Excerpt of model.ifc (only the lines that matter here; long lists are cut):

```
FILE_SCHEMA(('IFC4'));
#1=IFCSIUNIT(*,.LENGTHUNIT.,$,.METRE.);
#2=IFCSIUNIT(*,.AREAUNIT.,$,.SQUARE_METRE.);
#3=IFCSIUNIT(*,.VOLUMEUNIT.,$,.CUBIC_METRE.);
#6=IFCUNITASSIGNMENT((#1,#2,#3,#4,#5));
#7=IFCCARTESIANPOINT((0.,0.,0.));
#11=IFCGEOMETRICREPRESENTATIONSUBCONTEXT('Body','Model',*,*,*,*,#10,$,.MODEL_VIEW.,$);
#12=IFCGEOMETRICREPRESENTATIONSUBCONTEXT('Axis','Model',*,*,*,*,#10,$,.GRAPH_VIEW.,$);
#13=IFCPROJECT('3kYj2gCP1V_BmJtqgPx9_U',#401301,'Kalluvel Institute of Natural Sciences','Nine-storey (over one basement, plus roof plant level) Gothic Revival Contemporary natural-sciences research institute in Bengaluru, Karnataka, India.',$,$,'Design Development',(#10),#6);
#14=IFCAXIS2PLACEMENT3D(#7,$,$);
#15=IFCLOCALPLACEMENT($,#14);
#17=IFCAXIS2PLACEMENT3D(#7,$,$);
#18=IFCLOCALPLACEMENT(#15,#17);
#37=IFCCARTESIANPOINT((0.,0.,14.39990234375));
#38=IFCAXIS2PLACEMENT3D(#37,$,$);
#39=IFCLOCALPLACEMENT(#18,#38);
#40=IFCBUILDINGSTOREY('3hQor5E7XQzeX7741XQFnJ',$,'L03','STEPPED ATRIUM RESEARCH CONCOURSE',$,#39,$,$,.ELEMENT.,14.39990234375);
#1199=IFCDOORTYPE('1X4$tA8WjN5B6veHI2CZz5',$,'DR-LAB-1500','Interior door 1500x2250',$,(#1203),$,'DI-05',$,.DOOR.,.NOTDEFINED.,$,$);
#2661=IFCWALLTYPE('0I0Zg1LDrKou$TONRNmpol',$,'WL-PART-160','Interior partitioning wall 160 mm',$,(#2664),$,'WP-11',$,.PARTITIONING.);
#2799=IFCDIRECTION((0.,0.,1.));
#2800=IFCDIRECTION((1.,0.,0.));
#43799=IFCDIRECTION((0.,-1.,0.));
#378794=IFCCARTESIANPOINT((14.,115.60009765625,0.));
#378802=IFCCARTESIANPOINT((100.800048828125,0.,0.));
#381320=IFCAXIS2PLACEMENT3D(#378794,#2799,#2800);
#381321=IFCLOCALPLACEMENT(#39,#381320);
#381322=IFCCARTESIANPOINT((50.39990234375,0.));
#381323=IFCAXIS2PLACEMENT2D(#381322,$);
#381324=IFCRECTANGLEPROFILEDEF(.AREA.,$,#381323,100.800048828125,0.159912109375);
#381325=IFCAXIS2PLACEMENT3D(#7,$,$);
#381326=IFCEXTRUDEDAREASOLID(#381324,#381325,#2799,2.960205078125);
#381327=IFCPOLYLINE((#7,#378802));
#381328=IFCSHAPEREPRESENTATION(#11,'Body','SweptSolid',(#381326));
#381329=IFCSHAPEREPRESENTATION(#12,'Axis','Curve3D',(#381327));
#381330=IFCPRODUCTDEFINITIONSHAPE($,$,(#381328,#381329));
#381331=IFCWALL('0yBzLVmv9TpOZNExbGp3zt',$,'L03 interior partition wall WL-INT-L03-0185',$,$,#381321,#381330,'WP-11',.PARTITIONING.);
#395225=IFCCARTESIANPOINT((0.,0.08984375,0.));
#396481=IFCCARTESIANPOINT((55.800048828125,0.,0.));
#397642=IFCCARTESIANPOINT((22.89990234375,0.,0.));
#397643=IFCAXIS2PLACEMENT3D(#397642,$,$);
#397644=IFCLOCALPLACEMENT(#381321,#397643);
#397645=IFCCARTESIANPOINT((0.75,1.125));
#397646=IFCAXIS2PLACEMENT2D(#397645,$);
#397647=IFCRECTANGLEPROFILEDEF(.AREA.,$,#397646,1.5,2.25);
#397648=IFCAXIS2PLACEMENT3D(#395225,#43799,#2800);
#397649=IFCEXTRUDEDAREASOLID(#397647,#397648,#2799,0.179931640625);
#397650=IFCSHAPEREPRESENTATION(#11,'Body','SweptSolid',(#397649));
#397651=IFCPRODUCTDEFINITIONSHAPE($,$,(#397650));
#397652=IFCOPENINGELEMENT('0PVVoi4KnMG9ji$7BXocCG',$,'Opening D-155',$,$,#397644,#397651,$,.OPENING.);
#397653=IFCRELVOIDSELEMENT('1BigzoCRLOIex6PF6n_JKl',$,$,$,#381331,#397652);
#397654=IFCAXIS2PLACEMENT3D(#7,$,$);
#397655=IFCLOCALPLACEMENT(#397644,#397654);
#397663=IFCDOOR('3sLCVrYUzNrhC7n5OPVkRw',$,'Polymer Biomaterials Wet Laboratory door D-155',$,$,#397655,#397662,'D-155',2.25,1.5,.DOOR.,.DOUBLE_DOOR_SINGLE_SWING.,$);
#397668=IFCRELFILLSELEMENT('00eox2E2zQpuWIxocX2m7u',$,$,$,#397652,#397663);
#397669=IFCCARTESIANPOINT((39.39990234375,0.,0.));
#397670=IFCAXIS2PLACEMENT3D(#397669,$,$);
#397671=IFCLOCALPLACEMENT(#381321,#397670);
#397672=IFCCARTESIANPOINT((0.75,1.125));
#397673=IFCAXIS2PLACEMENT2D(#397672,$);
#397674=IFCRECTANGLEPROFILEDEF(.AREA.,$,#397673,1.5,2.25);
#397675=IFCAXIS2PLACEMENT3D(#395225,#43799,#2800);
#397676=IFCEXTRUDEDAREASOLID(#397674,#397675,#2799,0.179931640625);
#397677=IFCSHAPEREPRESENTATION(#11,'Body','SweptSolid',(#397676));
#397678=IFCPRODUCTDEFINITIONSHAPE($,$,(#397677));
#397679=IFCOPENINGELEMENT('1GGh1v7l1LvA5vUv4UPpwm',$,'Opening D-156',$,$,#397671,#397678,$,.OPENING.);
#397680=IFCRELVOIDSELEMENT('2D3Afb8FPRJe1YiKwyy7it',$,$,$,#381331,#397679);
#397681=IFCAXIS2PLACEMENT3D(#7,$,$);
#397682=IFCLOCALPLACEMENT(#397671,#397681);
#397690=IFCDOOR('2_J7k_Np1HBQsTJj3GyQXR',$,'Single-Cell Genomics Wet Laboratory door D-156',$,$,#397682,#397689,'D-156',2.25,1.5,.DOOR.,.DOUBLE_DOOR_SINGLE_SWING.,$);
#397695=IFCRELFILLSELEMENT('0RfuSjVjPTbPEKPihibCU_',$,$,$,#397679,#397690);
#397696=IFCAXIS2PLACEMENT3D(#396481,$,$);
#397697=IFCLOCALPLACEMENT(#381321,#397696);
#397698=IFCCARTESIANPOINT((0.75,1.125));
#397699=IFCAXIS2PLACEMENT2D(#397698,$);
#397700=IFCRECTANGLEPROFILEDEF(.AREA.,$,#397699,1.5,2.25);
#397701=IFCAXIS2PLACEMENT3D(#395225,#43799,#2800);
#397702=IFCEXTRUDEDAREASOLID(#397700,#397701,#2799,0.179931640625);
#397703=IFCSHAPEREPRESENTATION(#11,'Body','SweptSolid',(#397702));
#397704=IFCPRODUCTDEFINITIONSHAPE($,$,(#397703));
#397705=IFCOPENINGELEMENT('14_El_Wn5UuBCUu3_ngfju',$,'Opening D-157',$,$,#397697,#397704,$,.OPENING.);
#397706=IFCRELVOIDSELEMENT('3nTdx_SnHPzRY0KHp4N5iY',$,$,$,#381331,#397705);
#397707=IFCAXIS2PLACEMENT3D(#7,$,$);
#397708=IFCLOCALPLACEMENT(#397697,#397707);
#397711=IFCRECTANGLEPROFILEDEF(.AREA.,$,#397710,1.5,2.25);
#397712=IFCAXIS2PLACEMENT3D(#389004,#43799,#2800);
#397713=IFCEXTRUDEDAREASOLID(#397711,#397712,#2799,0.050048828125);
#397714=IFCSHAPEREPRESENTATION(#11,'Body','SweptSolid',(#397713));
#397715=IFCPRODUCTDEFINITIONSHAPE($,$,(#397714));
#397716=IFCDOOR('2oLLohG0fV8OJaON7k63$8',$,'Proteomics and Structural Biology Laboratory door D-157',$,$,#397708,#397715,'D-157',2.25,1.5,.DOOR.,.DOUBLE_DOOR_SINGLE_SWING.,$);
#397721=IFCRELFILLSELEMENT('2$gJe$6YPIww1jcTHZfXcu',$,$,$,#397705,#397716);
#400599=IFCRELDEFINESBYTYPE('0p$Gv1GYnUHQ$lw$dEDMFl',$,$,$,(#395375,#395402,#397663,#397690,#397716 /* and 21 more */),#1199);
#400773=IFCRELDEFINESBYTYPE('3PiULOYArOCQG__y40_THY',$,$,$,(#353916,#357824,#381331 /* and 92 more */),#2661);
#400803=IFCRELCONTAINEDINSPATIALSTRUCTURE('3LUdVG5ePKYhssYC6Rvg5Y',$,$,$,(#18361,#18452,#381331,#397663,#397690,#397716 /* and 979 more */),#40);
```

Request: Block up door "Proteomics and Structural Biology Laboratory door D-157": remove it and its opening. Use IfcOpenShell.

```python
import ifcopenshell
import ifcopenshell.api.feature
import ifcopenshell.api.root
import ifcopenshell.geom
import ifcopenshell.util.shape

model = ifcopenshell.open("model.ifc")
settings = ifcopenshell.geom.settings()


def volume(element):
    """Net volume in cubic metres, openings subtracted."""
    shape = ifcopenshell.geom.create_shape(settings, element)
    return ifcopenshell.util.shape.get_volume(shape.geometry)


door = model.by_guid("2oLLohG0fV8OJaON7k63$8")
opening = door.FillsVoids[0].RelatingOpeningElement
wall = opening.VoidsElements[0].RelatingBuildingElement
before = volume(wall)

ifcopenshell.api.root.remove_product(model, product=door)
ifcopenshell.api.feature.remove_feature(model, feature=opening)

after = volume(wall)

print(f"wall volume {before:.3f} -> {after:.3f} m3")

model.write("model_edited.ifc")
```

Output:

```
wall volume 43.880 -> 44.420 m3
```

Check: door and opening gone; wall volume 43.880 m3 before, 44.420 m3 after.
